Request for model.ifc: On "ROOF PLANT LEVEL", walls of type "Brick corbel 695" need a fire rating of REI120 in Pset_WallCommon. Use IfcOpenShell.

First a look at what the model holds.

```python
import ifcopenshell
import ifcopenshell.util.element

model = ifcopenshell.open("model.ifc")
print(model.schema)
storey = next(s for s in model.by_type("IfcBuildingStorey") if s.Name == "ROOF PLANT LEVEL")
walls = [e for e in ifcopenshell.util.element.get_decomposition(storey) if e.is_a("IfcWall")]
seen = {}
for e in walls:
    element_type = ifcopenshell.util.element.get_type(e)
    key = (element_type.Name if element_type != e and element_type else None, ifcopenshell.util.element.get_pset(e, "Pset_WallCommon", "FireRating"))
    seen[key] = seen.get(key, 0) + 1
for (name, value), count in sorted(seen.items(), key=str):
    print(count, "x", name, "|", value)
```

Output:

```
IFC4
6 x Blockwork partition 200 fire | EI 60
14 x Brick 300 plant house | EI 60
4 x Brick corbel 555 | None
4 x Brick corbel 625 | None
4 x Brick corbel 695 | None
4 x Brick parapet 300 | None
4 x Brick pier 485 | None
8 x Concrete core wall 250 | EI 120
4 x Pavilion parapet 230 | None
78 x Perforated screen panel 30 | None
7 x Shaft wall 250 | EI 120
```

```python
import ifcopenshell
import ifcopenshell.api.pset
import ifcopenshell.util.element

model = ifcopenshell.open("model.ifc")

storey = next(s for s in model.by_type("IfcBuildingStorey") if s.Name == "ROOF PLANT LEVEL")
walls = [e for e in ifcopenshell.util.element.get_decomposition(storey) if e.is_a("IfcWall")]

count = 0
for e in walls:
    element_type = ifcopenshell.util.element.get_type(e)
    if element_type in (None, e) or element_type.Name != "Brick corbel 695":
        continue
    # add_pset returns the element's existing set when there is one.
    pset = ifcopenshell.api.pset.add_pset(model, product=e, name="Pset_WallCommon")
    ifcopenshell.api.pset.edit_pset(model, pset=pset, properties={"FireRating": "REI120"})
    count += 1

print(count, "walls updated")

model.write("model_edited.ifc")
```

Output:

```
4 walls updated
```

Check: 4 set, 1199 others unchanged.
